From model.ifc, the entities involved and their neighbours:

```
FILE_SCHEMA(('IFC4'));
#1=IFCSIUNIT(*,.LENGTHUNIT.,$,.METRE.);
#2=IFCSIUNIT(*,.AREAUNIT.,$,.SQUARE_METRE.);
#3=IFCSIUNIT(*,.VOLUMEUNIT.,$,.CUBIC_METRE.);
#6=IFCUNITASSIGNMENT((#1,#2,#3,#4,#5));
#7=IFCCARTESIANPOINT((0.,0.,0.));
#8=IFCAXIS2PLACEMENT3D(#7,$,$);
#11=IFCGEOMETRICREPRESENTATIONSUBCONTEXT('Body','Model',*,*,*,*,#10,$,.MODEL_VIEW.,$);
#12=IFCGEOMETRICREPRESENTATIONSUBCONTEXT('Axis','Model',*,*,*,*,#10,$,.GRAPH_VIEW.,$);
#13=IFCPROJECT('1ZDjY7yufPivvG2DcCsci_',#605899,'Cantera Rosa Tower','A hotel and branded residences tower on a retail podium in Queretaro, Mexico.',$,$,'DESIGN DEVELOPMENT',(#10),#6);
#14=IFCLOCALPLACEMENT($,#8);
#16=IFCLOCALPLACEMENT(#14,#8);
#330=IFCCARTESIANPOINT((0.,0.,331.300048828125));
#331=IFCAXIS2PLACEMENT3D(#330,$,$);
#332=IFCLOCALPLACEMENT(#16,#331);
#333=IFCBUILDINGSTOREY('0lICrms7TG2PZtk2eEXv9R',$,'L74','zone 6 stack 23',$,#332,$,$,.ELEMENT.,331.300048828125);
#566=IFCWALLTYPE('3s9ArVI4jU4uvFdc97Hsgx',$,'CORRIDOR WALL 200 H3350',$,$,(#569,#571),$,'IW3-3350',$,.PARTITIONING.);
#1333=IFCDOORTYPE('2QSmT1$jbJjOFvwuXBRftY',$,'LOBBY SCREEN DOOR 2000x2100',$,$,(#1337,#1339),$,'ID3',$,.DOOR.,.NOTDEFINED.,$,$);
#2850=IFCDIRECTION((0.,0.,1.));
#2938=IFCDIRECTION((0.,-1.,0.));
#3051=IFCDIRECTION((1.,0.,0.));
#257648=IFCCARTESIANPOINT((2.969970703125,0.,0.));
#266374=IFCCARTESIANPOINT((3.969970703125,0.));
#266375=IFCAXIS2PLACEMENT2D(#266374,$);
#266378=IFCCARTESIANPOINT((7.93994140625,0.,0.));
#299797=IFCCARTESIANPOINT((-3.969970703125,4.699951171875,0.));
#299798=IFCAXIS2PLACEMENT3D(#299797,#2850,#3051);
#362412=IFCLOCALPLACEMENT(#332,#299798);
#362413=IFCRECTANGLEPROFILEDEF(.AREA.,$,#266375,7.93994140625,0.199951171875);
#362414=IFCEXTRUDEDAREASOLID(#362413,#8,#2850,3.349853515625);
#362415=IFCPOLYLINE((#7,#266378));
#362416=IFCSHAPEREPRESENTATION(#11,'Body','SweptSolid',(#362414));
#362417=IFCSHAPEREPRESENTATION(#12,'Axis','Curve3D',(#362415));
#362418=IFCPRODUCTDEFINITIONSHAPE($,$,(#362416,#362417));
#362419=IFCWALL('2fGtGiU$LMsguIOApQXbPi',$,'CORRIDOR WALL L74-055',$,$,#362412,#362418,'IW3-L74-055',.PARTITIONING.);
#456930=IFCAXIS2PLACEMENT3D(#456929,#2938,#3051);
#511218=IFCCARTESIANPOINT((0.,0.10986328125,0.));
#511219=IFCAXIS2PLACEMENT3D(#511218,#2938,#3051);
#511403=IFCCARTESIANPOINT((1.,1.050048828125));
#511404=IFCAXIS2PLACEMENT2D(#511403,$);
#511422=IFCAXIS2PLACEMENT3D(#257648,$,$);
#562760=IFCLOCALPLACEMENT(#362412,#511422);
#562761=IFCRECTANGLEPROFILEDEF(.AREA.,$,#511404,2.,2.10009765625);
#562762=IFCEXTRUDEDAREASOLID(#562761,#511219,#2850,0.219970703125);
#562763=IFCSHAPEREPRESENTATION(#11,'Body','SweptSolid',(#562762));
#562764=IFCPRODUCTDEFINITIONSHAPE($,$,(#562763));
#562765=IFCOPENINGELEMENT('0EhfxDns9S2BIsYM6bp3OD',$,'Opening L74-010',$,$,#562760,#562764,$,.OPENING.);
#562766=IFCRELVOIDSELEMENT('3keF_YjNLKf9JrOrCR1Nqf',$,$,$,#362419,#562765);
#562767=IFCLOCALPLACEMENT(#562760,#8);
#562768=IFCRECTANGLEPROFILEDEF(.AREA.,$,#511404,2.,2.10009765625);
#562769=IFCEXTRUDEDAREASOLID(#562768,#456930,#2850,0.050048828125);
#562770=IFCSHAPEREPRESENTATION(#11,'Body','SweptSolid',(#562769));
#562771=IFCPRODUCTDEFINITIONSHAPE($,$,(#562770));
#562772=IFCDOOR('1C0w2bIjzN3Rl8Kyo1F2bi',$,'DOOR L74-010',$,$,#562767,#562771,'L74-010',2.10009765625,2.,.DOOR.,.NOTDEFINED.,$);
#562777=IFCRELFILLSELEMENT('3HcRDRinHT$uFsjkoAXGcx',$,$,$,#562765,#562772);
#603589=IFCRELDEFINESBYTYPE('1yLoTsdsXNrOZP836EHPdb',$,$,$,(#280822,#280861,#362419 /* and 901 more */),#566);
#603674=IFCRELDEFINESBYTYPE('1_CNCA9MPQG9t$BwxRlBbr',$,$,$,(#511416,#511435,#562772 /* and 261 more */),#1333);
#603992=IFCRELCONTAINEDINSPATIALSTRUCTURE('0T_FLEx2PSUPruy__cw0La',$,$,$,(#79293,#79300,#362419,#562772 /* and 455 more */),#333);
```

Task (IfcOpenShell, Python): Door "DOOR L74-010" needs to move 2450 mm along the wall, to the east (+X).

```python
import ifcopenshell
import ifcopenshell.api.geometry
import ifcopenshell.util.placement

model = ifcopenshell.open("model.ifc")

door = model.by_id(562772)
opening = door.FillsVoids[0].RelatingOpeningElement
wall = opening.VoidsElements[0].RelatingBuildingElement

wall_matrix = ifcopenshell.util.placement.get_local_placement(wall.ObjectPlacement)
shift = wall_matrix[:3, 0] * 2.45
before = ifcopenshell.util.placement.get_local_placement(door.ObjectPlacement)[:3, 3].copy()

# The door is placed relative to its opening, so it follows when the opening moves.
matrix = ifcopenshell.util.placement.get_local_placement(opening.ObjectPlacement)
matrix[:3, 3] += shift
ifcopenshell.api.geometry.edit_object_placement(
    model, product=opening, matrix=matrix, is_si=False, should_transform_children=True
)

after = ifcopenshell.util.placement.get_local_placement(door.ObjectPlacement)[:3, 3]
print("door moved by", (after - before).round(3) + 0.0)

model.write("model_updated.ifc")
```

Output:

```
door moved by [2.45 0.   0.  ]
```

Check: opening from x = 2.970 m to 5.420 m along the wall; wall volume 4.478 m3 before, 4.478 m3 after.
